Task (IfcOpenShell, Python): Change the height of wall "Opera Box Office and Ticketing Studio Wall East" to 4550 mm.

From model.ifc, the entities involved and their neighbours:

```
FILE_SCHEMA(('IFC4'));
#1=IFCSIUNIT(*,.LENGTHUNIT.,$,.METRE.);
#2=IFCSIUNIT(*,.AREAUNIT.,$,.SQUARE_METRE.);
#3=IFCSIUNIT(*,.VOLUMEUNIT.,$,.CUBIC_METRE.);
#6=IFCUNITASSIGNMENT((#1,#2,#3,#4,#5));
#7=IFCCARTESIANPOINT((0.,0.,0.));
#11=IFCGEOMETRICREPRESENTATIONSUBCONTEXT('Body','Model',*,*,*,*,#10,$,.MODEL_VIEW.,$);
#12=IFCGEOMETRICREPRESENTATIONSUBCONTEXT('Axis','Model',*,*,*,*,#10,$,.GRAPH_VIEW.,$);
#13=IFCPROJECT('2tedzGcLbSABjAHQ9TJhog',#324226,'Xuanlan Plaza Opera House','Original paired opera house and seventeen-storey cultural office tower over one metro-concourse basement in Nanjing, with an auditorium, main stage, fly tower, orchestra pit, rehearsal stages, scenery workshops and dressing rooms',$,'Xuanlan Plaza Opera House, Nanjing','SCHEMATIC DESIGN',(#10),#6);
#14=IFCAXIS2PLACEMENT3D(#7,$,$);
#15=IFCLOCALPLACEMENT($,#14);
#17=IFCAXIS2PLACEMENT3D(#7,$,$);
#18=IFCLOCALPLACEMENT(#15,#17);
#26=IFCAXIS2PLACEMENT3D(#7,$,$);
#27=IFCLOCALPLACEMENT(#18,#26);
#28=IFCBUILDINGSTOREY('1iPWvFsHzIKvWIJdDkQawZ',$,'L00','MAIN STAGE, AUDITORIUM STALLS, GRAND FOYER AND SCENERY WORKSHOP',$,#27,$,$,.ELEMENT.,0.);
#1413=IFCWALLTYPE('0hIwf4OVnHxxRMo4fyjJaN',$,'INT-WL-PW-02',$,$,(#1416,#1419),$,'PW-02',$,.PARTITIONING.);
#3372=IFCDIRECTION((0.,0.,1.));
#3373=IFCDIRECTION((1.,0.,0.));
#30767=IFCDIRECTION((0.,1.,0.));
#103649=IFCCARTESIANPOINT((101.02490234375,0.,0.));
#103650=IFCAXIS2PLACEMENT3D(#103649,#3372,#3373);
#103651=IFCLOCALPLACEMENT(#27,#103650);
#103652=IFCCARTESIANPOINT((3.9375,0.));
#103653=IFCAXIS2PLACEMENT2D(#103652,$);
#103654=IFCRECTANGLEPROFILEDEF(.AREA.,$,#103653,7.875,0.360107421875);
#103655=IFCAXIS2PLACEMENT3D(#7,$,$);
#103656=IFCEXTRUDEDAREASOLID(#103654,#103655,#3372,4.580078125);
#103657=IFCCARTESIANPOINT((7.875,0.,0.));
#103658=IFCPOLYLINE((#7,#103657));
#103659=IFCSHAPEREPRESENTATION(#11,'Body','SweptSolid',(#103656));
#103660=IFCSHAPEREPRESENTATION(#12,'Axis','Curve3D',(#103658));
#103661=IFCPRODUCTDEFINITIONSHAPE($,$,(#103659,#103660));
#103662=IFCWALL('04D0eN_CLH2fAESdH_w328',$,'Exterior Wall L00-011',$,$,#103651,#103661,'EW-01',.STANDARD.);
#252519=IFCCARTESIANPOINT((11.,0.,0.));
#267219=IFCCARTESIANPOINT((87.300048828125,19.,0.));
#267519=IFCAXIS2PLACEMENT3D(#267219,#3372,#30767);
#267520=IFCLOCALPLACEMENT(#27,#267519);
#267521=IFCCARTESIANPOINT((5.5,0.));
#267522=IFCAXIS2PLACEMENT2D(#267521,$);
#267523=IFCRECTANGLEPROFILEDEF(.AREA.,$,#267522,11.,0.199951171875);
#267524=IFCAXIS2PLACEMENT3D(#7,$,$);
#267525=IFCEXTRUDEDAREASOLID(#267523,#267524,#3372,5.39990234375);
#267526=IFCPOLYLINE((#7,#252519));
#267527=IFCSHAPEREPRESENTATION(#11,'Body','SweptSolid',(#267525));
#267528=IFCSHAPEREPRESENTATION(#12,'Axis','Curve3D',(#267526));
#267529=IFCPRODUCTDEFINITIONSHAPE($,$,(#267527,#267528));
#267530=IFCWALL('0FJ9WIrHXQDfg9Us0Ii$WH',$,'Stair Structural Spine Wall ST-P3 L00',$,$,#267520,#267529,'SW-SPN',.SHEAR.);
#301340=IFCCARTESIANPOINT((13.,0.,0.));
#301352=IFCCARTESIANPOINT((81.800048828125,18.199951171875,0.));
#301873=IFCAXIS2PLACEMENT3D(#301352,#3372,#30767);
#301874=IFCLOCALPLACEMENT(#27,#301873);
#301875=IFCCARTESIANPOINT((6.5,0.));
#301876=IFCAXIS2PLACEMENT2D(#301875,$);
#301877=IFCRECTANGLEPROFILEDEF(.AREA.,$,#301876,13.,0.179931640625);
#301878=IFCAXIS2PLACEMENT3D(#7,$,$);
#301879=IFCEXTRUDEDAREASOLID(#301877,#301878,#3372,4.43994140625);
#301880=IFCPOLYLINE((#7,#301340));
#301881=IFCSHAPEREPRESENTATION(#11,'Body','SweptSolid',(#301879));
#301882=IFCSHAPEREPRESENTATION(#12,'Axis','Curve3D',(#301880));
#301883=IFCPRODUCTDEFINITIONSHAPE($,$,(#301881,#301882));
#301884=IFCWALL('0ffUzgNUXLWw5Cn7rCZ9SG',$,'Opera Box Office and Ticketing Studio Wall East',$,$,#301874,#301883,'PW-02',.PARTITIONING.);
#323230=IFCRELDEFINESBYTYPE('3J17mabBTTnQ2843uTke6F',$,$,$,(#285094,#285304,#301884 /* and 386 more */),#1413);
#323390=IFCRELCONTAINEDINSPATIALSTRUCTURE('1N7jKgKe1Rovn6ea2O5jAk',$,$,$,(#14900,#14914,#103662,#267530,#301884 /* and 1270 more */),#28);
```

```python
import ifcopenshell
import ifcopenshell.geom
import ifcopenshell.util.representation
import ifcopenshell.util.shape

model = ifcopenshell.open("model.ifc")
settings = ifcopenshell.geom.settings()


def volume(element):
    """Net volume in cubic metres, openings subtracted."""
    shape = ifcopenshell.geom.create_shape(settings, element)
    return ifcopenshell.util.shape.get_volume(shape.geometry)


wall = model.by_guid("0ffUzgNUXLWw5Cn7rCZ9SG")
before = volume(wall)

body = ifcopenshell.util.representation.get_representation(wall, "Model", "Body")
solid = body.Items[0]
old_height = solid.Depth
solid.Depth = 4.55
after = volume(wall)

print(f"height {old_height:g} -> {solid.Depth:g}, volume {before:.3f} -> {after:.3f} m3")

model.write("model-out.ifc")
```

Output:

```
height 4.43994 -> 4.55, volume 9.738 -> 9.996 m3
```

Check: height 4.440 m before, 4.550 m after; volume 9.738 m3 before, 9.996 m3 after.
